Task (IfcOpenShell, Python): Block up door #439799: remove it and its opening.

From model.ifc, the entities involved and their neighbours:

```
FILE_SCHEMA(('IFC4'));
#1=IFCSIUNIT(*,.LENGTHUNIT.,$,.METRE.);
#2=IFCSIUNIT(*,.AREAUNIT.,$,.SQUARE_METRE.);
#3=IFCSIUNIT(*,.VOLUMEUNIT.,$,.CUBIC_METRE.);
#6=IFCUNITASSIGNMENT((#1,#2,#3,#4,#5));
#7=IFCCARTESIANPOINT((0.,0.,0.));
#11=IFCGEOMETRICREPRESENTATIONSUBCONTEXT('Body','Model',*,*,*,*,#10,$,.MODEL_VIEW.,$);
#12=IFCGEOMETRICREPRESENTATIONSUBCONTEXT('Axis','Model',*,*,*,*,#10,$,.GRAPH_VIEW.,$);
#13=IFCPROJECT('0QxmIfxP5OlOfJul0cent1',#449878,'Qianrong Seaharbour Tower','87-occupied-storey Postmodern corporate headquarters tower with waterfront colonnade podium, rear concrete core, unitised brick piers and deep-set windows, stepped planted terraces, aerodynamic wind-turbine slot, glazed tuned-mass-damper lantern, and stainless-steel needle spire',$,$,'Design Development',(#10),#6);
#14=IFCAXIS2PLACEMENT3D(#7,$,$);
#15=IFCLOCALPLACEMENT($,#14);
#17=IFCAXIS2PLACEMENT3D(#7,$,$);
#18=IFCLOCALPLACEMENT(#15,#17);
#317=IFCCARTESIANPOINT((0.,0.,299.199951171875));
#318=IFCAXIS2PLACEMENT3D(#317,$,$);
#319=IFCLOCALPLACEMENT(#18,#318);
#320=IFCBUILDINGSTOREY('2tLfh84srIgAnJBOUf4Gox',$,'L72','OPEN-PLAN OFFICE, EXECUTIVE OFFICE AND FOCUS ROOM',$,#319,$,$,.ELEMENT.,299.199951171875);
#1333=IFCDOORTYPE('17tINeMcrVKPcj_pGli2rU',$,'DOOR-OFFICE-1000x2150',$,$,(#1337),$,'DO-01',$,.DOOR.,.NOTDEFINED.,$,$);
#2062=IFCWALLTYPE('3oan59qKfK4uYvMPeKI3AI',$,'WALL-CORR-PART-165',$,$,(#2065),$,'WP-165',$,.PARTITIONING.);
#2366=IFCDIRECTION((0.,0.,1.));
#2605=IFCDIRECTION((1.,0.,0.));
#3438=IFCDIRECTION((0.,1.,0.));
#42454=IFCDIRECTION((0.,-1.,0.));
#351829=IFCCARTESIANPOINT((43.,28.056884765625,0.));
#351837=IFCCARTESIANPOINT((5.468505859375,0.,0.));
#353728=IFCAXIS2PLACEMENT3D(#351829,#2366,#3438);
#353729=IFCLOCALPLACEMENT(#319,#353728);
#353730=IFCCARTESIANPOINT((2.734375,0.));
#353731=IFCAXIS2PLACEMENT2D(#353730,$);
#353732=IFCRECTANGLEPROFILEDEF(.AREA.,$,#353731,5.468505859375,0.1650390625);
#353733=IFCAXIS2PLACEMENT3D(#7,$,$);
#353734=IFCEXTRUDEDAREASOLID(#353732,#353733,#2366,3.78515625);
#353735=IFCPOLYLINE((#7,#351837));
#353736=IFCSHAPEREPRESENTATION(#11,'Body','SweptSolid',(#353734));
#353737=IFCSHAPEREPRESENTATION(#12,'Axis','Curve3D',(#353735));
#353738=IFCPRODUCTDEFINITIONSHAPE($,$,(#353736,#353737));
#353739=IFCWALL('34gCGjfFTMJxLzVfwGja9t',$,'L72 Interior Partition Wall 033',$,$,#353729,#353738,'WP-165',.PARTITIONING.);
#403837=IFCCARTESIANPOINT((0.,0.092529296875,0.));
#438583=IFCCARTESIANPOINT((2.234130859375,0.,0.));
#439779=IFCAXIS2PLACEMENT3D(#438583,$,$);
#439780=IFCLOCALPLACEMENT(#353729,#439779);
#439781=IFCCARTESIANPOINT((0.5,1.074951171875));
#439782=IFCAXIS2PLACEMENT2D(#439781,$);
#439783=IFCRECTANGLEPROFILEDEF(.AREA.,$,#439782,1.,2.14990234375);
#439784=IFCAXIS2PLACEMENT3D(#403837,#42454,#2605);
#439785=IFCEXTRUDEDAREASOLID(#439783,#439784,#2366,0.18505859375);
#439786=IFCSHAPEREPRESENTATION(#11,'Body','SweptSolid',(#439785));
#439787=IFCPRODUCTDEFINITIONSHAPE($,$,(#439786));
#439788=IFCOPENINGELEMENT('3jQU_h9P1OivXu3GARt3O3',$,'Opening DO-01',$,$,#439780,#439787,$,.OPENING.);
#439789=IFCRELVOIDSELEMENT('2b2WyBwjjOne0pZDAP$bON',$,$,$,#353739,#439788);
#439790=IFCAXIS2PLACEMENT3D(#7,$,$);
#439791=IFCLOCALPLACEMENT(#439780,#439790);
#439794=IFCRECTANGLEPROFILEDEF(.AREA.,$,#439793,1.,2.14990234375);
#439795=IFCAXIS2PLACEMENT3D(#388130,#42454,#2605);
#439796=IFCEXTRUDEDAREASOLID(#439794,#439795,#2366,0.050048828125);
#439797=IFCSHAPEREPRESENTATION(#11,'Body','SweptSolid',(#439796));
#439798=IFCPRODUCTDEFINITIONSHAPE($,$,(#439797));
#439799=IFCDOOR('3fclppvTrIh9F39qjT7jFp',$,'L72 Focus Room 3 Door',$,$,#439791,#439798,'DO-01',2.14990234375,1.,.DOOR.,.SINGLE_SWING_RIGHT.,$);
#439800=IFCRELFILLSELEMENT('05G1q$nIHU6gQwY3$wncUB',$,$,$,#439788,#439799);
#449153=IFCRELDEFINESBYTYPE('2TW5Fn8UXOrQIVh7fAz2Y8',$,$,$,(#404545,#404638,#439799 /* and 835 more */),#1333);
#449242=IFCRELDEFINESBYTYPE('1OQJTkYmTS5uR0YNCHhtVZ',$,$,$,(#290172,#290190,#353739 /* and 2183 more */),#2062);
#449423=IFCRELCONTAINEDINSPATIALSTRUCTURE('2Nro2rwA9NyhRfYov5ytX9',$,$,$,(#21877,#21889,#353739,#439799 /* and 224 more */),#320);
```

```python
import ifcopenshell
import ifcopenshell.api.feature
import ifcopenshell.api.root
import ifcopenshell.geom
import ifcopenshell.util.shape

model = ifcopenshell.open("model.ifc")
settings = ifcopenshell.geom.settings()


def volume(element):
    """Net volume in cubic metres, openings subtracted."""
    shape = ifcopenshell.geom.create_shape(settings, element)
    return ifcopenshell.util.shape.get_volume(shape.geometry)


door = model.by_guid("3fclppvTrIh9F39qjT7jFp")
opening = door.FillsVoids[0].RelatingOpeningElement
wall = opening.VoidsElements[0].RelatingBuildingElement
before = volume(wall)

ifcopenshell.api.root.remove_product(model, product=door)
ifcopenshell.api.feature.remove_feature(model, feature=opening)

after = volume(wall)

print(f"wall volume {before:.3f} -> {after:.3f} m3")

model.write("model_rev.ifc")
```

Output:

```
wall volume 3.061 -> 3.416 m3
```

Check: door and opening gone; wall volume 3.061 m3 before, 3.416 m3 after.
